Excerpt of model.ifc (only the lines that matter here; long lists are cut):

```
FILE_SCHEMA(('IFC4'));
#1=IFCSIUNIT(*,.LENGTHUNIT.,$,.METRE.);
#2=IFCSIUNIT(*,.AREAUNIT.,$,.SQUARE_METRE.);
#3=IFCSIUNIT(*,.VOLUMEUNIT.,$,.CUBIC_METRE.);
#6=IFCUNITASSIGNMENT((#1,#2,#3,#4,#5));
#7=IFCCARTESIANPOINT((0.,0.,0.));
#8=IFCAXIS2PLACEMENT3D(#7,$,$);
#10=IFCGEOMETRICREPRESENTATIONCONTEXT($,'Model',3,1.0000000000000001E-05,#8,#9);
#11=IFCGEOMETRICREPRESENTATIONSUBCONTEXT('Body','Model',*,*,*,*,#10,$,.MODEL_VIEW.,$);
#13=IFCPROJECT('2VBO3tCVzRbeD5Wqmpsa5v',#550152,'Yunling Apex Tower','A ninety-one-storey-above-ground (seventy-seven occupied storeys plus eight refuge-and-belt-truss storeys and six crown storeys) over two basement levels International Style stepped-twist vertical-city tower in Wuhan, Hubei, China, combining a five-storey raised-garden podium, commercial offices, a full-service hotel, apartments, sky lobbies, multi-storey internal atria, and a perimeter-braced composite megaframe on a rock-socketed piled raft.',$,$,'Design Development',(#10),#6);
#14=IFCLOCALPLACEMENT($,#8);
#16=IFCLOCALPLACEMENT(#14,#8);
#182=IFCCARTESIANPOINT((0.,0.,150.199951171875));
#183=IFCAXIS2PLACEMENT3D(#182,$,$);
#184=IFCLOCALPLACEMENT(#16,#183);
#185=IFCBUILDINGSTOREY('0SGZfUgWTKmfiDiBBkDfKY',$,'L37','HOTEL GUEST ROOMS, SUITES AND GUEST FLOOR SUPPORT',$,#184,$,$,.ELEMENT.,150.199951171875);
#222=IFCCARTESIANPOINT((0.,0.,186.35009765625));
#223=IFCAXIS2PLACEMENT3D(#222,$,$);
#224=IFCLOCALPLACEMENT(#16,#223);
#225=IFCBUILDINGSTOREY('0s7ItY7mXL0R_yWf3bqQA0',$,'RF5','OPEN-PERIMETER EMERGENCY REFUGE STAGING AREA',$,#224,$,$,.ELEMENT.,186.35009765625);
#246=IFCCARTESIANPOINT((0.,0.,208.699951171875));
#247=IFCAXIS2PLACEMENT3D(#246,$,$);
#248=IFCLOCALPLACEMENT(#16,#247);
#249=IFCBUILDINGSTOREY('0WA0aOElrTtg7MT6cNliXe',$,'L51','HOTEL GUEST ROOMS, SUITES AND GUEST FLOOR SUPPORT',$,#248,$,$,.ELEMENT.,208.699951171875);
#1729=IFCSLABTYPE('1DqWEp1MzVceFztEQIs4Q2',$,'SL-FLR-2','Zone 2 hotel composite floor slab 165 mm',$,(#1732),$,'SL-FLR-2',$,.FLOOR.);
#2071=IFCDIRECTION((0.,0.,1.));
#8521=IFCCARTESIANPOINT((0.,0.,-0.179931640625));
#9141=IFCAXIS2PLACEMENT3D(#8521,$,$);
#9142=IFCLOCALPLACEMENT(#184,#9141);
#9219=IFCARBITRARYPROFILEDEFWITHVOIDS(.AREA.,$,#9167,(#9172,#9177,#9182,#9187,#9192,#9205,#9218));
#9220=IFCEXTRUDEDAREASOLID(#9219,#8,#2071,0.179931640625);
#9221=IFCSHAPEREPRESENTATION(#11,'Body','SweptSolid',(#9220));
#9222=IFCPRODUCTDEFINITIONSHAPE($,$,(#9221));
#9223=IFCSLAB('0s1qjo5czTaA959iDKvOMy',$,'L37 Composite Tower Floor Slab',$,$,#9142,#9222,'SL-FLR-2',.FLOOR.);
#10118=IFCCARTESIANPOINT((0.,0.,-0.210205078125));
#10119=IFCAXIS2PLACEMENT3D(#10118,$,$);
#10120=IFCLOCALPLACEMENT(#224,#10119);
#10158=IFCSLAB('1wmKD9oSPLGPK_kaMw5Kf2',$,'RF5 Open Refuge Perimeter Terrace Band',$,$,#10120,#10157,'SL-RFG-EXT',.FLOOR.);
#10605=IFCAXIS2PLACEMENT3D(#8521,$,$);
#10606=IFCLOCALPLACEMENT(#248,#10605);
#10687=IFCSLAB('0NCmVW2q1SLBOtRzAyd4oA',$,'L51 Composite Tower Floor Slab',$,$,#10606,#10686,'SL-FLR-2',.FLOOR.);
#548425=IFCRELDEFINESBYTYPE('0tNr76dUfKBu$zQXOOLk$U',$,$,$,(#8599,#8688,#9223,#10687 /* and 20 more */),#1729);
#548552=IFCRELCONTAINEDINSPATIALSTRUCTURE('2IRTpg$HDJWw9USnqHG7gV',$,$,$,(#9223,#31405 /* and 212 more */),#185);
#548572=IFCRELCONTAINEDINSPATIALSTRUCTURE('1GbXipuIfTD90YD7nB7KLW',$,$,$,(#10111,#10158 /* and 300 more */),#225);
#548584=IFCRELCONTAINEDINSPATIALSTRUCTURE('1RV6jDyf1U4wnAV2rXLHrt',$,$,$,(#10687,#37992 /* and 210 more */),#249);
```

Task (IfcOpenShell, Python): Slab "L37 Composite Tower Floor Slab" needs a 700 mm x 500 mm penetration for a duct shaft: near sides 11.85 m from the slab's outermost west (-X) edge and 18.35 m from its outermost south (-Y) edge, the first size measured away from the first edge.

```python
import numpy as np
import ifcopenshell
import ifcopenshell.api.feature
import ifcopenshell.api.geometry
import ifcopenshell.api.root
import ifcopenshell.geom
import ifcopenshell.util.placement
import ifcopenshell.util.representation
import ifcopenshell.util.shape
import ifcopenshell.util.unit

model = ifcopenshell.open("model.ifc")
unit_scale = ifcopenshell.util.unit.calculate_unit_scale(model)
settings = ifcopenshell.geom.settings()


def volume(element):
    """Net volume in cubic metres, openings subtracted."""
    shape = ifcopenshell.geom.create_shape(settings, element)
    return ifcopenshell.util.shape.get_volume(shape.geometry)


slab = model.by_guid("0s1qjo5czTaA959iDKvOMy")
before = volume(slab)

# Extent in the slab's own axes, in metres. The edges named are its -X and -Y sides.
slab_shape = ifcopenshell.geom.create_shape(settings, slab)
vertices = ifcopenshell.util.shape.get_vertices(slab_shape.geometry)
x_min, y_min, bottom = vertices.min(axis=0)
top = vertices[:, 2].max()

opening = ifcopenshell.api.root.create_entity(model, ifc_class="IfcOpeningElement", name="Duct shaft opening", predefined_type="OPENING")
context = ifcopenshell.util.representation.get_context(model, "Model", "Body", "MODEL_VIEW")
width, depth = 0.7, 0.5
outline = [(0.0, 0.0), (width, 0.0), (width, depth), (0.0, depth), (0.0, 0.0)]
# Overshoot both faces by 50 mm so the cut is clean.
shape = ifcopenshell.api.geometry.add_slab_representation(
    model, context=context, depth=top - bottom + 0.1, polyline=outline
)
ifcopenshell.api.geometry.assign_representation(model, product=opening, representation=shape)

matrix = ifcopenshell.util.placement.get_local_placement(slab.ObjectPlacement)
matrix[:, 3] = matrix @ np.append(np.array([x_min + 11.85, y_min + 18.35, bottom - 0.05]) / unit_scale, 1.0)
ifcopenshell.api.geometry.edit_object_placement(model, product=opening, matrix=matrix, is_si=False)
ifcopenshell.api.feature.add_feature(model, feature=opening, element=slab)

after = volume(slab)

print(f"slab volume {before:.3f} -> {after:.3f} m3")

model.write("model_edited.ifc")
```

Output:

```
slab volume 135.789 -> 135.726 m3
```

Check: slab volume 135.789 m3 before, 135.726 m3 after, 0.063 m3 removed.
